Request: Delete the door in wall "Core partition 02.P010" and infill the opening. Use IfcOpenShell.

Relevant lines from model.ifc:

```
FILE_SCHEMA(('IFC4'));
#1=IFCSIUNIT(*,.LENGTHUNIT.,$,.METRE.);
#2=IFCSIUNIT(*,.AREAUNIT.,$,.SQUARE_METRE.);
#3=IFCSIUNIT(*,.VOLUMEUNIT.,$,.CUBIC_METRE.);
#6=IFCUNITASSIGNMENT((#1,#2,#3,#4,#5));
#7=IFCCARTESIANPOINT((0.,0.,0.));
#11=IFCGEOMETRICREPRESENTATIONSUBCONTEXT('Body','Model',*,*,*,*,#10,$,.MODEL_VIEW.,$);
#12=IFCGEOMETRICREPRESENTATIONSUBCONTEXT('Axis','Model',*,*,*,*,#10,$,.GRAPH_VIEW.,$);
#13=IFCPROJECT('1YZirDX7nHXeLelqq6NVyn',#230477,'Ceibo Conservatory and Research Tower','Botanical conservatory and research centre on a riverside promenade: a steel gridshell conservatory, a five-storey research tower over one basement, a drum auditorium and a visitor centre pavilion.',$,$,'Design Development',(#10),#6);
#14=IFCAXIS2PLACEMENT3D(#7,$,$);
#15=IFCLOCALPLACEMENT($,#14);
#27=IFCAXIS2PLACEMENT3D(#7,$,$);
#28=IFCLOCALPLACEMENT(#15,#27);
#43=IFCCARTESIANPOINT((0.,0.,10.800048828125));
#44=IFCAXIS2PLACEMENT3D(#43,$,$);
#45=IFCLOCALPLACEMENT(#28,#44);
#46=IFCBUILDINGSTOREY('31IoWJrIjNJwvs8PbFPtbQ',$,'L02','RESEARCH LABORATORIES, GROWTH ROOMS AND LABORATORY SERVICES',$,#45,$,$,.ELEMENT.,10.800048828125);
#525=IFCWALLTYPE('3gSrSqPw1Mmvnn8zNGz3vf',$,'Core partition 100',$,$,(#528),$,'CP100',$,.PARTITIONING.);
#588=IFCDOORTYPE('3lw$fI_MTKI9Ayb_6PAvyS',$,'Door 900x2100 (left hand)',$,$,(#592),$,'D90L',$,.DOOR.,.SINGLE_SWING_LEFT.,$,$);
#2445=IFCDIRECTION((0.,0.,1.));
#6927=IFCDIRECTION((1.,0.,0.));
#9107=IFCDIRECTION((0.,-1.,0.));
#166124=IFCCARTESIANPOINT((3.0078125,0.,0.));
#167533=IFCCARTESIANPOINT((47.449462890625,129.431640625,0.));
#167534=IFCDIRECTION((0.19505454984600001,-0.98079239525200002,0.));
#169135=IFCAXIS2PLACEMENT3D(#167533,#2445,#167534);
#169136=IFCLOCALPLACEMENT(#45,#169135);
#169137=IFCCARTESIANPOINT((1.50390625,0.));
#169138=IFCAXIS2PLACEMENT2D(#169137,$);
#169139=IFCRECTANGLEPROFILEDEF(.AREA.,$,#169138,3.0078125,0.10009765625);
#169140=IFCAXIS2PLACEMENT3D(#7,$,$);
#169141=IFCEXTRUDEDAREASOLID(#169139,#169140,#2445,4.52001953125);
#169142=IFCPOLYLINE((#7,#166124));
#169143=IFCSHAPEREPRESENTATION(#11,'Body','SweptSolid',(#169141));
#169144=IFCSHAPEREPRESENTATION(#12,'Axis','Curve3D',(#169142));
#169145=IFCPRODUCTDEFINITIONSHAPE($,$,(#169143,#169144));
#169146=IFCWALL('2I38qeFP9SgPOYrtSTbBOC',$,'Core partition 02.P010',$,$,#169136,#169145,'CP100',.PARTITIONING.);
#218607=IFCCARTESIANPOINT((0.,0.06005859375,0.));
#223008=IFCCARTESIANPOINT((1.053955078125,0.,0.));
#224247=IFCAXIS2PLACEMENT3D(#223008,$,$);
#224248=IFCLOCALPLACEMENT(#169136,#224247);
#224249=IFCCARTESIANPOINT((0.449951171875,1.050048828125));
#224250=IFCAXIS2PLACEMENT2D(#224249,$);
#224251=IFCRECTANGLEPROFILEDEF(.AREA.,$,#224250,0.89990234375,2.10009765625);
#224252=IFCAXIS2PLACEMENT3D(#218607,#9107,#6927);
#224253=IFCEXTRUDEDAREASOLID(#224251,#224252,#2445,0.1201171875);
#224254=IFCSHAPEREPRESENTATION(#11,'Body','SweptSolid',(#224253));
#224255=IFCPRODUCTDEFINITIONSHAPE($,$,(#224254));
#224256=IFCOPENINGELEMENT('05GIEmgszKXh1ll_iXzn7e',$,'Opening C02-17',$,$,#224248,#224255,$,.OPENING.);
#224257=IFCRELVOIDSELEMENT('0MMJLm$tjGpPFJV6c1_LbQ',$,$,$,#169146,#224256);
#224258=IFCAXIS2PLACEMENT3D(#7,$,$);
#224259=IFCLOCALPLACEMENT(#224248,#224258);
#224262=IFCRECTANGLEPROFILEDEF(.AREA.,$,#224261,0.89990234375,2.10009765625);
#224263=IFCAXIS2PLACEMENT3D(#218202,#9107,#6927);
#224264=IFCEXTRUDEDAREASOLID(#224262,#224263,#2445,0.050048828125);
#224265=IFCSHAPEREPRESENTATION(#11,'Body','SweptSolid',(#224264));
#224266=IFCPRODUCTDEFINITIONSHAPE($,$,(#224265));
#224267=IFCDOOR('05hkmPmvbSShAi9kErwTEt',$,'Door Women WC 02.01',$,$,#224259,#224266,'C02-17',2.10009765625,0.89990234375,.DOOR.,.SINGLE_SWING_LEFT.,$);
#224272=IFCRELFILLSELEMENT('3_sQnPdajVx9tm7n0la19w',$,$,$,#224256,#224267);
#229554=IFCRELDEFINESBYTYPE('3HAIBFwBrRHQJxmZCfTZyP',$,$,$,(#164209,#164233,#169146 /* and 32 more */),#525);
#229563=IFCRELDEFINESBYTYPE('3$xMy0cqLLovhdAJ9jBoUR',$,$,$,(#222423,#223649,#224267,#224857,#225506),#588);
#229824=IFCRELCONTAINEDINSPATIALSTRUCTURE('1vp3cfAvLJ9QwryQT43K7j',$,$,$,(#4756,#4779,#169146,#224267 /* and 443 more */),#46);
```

```python
import ifcopenshell
import ifcopenshell.api.feature
import ifcopenshell.api.root
import ifcopenshell.geom
import ifcopenshell.util.shape

model = ifcopenshell.open("model.ifc")
settings = ifcopenshell.geom.settings()


def volume(element):
    """Net volume in cubic metres, openings subtracted."""
    shape = ifcopenshell.geom.create_shape(settings, element)
    return ifcopenshell.util.shape.get_volume(shape.geometry)


door = model.by_guid("05hkmPmvbSShAi9kErwTEt")
opening = door.FillsVoids[0].RelatingOpeningElement
wall = opening.VoidsElements[0].RelatingBuildingElement
before = volume(wall)

ifcopenshell.api.root.remove_product(model, product=door)
ifcopenshell.api.feature.remove_feature(model, feature=opening)

after = volume(wall)

print(f"wall volume {before:.3f} -> {after:.3f} m3")

model.write("model_v2.ifc")
```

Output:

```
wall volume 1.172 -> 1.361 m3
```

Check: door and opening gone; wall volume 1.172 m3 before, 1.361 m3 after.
